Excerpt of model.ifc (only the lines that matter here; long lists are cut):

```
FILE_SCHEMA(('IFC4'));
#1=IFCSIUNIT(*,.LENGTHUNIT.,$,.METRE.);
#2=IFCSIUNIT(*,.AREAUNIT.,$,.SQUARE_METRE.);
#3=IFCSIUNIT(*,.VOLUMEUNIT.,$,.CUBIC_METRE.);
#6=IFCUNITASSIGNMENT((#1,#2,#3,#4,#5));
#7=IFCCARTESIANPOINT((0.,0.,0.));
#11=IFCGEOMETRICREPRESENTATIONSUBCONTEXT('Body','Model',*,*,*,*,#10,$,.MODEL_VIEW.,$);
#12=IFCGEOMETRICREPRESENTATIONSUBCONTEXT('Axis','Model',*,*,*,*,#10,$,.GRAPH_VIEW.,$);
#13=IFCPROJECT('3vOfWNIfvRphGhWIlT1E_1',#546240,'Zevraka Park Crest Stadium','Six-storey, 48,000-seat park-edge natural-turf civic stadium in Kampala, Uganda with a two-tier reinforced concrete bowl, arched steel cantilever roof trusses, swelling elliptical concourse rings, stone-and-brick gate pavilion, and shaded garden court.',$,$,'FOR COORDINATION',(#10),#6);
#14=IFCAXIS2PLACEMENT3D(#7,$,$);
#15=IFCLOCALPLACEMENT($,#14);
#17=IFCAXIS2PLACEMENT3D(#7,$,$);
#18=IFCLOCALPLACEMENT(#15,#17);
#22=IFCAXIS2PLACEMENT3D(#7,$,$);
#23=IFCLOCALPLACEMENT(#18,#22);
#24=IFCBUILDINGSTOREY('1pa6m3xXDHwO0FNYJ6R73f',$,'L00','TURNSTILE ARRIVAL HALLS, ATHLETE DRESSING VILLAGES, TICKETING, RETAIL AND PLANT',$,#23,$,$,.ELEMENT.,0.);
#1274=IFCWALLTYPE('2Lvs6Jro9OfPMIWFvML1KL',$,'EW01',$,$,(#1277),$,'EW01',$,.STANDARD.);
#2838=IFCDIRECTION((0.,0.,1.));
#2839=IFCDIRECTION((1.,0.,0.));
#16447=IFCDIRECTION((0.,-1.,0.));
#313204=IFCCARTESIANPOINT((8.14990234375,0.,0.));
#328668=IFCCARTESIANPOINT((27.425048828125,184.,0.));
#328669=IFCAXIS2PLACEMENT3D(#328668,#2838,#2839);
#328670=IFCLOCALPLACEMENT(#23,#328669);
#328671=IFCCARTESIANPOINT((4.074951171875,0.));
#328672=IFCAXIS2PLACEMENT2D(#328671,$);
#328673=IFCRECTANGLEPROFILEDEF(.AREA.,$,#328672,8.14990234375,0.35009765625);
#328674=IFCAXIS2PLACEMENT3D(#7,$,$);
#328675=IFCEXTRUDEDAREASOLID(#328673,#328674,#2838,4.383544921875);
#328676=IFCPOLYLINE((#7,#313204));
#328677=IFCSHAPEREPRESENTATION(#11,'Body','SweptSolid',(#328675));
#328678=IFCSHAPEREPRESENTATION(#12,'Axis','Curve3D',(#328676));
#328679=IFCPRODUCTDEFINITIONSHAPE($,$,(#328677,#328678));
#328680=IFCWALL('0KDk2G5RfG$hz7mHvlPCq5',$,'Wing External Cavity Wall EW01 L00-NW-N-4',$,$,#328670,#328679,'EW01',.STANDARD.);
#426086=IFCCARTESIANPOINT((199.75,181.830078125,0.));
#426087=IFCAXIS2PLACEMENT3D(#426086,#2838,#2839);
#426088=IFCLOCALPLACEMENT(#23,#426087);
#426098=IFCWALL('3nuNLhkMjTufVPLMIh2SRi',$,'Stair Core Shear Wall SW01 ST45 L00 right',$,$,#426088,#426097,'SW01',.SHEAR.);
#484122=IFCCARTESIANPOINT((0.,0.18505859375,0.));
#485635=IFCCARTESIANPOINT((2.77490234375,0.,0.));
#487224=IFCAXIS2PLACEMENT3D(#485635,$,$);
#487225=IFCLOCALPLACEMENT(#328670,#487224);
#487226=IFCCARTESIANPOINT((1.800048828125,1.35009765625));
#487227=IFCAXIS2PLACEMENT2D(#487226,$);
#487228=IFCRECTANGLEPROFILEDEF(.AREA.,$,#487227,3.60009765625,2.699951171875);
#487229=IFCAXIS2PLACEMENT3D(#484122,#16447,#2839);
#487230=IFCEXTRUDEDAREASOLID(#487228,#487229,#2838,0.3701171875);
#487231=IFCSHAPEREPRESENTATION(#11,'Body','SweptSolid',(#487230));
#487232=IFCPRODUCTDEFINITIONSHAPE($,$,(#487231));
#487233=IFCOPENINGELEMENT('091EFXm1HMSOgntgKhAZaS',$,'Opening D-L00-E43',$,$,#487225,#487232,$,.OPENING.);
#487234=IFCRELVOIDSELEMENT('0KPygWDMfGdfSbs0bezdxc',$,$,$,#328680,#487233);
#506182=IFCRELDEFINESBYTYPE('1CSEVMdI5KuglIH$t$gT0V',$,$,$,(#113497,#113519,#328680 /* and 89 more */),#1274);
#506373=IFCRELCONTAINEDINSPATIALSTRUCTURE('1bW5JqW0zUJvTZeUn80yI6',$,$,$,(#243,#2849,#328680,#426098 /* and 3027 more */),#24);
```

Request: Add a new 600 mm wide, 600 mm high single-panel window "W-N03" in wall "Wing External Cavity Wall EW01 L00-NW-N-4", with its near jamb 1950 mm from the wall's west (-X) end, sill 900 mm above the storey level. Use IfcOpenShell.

```python
import numpy as np
import ifcopenshell
import ifcopenshell.api.feature
import ifcopenshell.api.geometry
import ifcopenshell.api.root
import ifcopenshell.api.spatial
import ifcopenshell.geom
import ifcopenshell.util.element
import ifcopenshell.util.placement
import ifcopenshell.util.representation
import ifcopenshell.util.shape
import ifcopenshell.util.unit

model = ifcopenshell.open("model.ifc")
unit_scale = ifcopenshell.util.unit.calculate_unit_scale(model)
settings = ifcopenshell.geom.settings()


def volume(element):
    """Net volume in cubic metres, openings subtracted."""
    shape = ifcopenshell.geom.create_shape(settings, element)
    return ifcopenshell.util.shape.get_volume(shape.geometry)


wall = model.by_guid("0KDk2G5RfG$hz7mHvlPCq5")
storey = ifcopenshell.util.element.get_container(wall, ifc_class="IfcBuildingStorey")
context = ifcopenshell.util.representation.get_context(model, "Model", "Body", "MODEL_VIEW")
before = volume(wall)

width, height, from_end, sill = 0.6, 0.6, 1.95, 0.9  # metres

# The wall runs along its own X axis, and the end named is its -X end.
wall_shape = ifcopenshell.geom.create_shape(settings, wall)
x, y, z = ifcopenshell.util.shape.get_vertices(wall_shape.geometry).T
start = x.min() + from_end
face, thickness = float(y.min()), float(y.max() - y.min())
wall_matrix = ifcopenshell.util.placement.get_local_placement(wall.ObjectPlacement)
level = ifcopenshell.util.placement.get_local_placement(storey.ObjectPlacement)[2, 3]


def in_wall(x, y):
    """Placement at x, y metres in the wall's axes, at sill height."""
    matrix = wall_matrix.copy()
    matrix[:, 3] = wall_matrix @ np.array([x / unit_scale, y / unit_scale, 0.0, 1.0])
    matrix[2, 3] = level + sill / unit_scale
    return matrix


# Opening: a box that overshoots both wall faces by 50 mm.
opening = ifcopenshell.api.root.create_entity(model, ifc_class="IfcOpeningElement", predefined_type="OPENING")
box = ifcopenshell.api.geometry.add_wall_representation(
    model, context=context, length=width, height=height, thickness=thickness + 0.1
)
ifcopenshell.api.geometry.assign_representation(model, product=opening, representation=box)
ifcopenshell.api.geometry.edit_object_placement(model, product=opening, matrix=in_wall(start, face - 0.05), is_si=False)
ifcopenshell.api.feature.add_feature(model, feature=opening, element=wall)

window = ifcopenshell.api.root.create_entity(model, ifc_class="IfcWindow", name="W-N03", predefined_type="WINDOW")
window.OverallWidth, window.OverallHeight = width / unit_scale, height / unit_scale
window.PartitioningType = "SINGLE_PANEL"
body = ifcopenshell.api.geometry.add_window_representation(
    model,
    context=context,
    overall_width=window.OverallWidth,
    overall_height=window.OverallHeight,
    partition_type="SINGLE_PANEL",
)
ifcopenshell.api.geometry.assign_representation(model, product=window, representation=body)
ifcopenshell.api.spatial.assign_container(model, products=[window], relating_structure=storey)
ifcopenshell.api.feature.add_filling(model, opening=opening, element=window)

# Centre the window in the wall's thickness.
ifcopenshell.api.geometry.edit_object_placement(model, product=window, matrix=in_wall(start, face), is_si=False)
window_shape = ifcopenshell.geom.create_shape(settings, window)
depth = ifcopenshell.util.shape.get_vertices(window_shape.geometry)[:, 1]
offset = face + thickness / 2 - (depth.min() + depth.max()) / 2
ifcopenshell.api.geometry.edit_object_placement(model, product=window, matrix=in_wall(start, offset), is_si=False)

after = volume(wall)

print(f"wall volume {before:.3f} -> {after:.3f} m3")

model.write("model_v2.ifc")
```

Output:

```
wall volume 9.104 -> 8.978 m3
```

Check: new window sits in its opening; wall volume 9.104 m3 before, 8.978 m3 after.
